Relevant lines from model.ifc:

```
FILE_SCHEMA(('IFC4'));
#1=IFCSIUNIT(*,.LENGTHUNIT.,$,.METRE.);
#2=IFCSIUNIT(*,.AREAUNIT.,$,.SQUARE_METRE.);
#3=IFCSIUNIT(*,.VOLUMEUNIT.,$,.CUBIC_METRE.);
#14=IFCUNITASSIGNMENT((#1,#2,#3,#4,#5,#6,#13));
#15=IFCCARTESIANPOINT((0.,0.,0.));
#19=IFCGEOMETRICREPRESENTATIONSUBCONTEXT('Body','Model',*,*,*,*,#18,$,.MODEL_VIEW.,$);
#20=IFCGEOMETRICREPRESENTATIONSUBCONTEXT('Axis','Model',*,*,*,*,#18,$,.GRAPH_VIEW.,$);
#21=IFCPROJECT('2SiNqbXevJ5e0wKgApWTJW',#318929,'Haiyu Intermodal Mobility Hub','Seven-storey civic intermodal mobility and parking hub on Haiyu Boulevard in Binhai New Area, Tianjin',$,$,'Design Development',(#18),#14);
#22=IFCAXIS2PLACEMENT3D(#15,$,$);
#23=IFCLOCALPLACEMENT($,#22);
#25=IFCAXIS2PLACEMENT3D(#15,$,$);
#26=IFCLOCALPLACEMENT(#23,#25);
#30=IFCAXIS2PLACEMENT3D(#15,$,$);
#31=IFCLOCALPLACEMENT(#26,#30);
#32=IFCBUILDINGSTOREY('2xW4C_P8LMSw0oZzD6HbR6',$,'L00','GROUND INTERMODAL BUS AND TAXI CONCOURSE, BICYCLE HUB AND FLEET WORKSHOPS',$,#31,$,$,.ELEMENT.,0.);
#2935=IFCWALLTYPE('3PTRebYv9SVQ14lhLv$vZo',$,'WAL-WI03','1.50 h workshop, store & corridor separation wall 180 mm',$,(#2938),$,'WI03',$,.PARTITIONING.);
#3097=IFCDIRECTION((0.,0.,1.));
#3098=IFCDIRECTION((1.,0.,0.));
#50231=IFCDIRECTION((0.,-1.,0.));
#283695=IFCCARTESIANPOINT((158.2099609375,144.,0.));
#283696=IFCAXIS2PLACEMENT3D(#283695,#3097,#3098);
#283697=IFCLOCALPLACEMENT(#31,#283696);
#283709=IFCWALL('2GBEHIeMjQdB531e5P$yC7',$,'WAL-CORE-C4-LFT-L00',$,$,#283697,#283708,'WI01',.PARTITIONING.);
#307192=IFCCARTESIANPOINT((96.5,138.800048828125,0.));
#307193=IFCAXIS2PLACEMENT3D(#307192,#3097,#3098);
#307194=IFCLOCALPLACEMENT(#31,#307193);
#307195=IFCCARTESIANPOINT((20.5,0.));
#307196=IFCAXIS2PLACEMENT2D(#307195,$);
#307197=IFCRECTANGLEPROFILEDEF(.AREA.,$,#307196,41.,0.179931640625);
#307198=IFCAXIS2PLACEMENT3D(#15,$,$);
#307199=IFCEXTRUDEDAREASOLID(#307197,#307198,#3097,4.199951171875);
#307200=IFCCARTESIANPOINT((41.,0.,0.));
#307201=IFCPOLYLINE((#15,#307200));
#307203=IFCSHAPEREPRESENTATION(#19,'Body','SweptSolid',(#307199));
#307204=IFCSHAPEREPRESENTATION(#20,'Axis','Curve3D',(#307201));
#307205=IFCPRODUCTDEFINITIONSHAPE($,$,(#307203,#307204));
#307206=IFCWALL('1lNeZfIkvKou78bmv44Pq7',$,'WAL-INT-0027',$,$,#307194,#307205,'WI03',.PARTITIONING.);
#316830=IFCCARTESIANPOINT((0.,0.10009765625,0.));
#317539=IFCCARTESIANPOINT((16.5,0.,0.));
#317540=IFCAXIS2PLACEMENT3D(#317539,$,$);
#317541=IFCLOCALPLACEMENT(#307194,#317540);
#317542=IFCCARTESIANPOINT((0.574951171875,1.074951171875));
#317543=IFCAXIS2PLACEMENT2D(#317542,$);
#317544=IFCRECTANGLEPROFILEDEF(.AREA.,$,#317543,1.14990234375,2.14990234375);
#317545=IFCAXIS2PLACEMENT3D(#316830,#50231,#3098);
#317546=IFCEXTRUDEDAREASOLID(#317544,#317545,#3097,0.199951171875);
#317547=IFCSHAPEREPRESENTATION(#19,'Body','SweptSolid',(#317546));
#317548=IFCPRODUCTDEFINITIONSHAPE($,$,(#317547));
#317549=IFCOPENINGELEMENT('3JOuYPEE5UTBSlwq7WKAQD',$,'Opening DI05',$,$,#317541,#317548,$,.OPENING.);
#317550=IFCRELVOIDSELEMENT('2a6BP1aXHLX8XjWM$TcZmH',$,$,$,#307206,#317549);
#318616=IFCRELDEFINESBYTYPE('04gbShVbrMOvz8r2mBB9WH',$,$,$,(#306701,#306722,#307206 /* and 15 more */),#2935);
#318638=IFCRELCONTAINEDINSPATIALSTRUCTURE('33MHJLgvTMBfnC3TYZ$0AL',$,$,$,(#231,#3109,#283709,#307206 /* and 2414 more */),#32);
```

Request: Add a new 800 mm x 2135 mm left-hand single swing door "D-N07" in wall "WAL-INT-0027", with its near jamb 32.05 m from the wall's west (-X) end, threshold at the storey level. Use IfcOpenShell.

```python
import numpy as np
import ifcopenshell
import ifcopenshell.api.feature
import ifcopenshell.api.geometry
import ifcopenshell.api.root
import ifcopenshell.api.spatial
import ifcopenshell.geom
import ifcopenshell.util.element
import ifcopenshell.util.placement
import ifcopenshell.util.representation
import ifcopenshell.util.shape
import ifcopenshell.util.unit

model = ifcopenshell.open("model.ifc")
unit_scale = ifcopenshell.util.unit.calculate_unit_scale(model)
settings = ifcopenshell.geom.settings()


def volume(element):
    """Net volume in cubic metres, openings subtracted."""
    shape = ifcopenshell.geom.create_shape(settings, element)
    return ifcopenshell.util.shape.get_volume(shape.geometry)


wall = model.by_guid("1lNeZfIkvKou78bmv44Pq7")
storey = ifcopenshell.util.element.get_container(wall, ifc_class="IfcBuildingStorey")
context = ifcopenshell.util.representation.get_context(model, "Model", "Body", "MODEL_VIEW")
before = volume(wall)

width, height, from_end, sill = 0.8, 2.135, 32.05, 0.0  # metres

# The wall runs along its own X axis, and the end named is its -X end.
wall_shape = ifcopenshell.geom.create_shape(settings, wall)
x, y, z = ifcopenshell.util.shape.get_vertices(wall_shape.geometry).T
start = x.min() + from_end
face, thickness = float(y.min()), float(y.max() - y.min())
wall_matrix = ifcopenshell.util.placement.get_local_placement(wall.ObjectPlacement)
level = ifcopenshell.util.placement.get_local_placement(storey.ObjectPlacement)[2, 3]


def in_wall(x, y):
    """Placement at x, y metres in the wall's axes, at sill height."""
    matrix = wall_matrix.copy()
    matrix[:, 3] = wall_matrix @ np.array([x / unit_scale, y / unit_scale, 0.0, 1.0])
    matrix[2, 3] = level + sill / unit_scale
    return matrix


# Opening: a box that overshoots both wall faces by 50 mm.
opening = ifcopenshell.api.root.create_entity(model, ifc_class="IfcOpeningElement", predefined_type="OPENING")
box = ifcopenshell.api.geometry.add_wall_representation(
    model, context=context, length=width, height=height, thickness=thickness + 0.1
)
ifcopenshell.api.geometry.assign_representation(model, product=opening, representation=box)
ifcopenshell.api.geometry.edit_object_placement(model, product=opening, matrix=in_wall(start, face - 0.05), is_si=False)
ifcopenshell.api.feature.add_feature(model, feature=opening, element=wall)

door = ifcopenshell.api.root.create_entity(model, ifc_class="IfcDoor", name="D-N07", predefined_type="DOOR")
door.OverallWidth, door.OverallHeight = width / unit_scale, height / unit_scale
door.OperationType = "SINGLE_SWING_LEFT"
body = ifcopenshell.api.geometry.add_door_representation(
    model,
    context=context,
    overall_width=door.OverallWidth,
    overall_height=door.OverallHeight,
    operation_type="SINGLE_SWING_LEFT",
    lining_properties={"LiningDepth": thickness / unit_scale, "ThresholdDepth": thickness / unit_scale},
)
ifcopenshell.api.geometry.assign_representation(model, product=door, representation=body)
ifcopenshell.api.spatial.assign_container(model, products=[door], relating_structure=storey)
ifcopenshell.api.feature.add_filling(model, opening=opening, element=door)

# The lining spans the wall, so the door starts at the wall face.
ifcopenshell.api.geometry.edit_object_placement(model, product=door, matrix=in_wall(start, face), is_si=False)

after = volume(wall)

print(f"wall volume {before:.3f} -> {after:.3f} m3")

model.write("model-out.ifc")
```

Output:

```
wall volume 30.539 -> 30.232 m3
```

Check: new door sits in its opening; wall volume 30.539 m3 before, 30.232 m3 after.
